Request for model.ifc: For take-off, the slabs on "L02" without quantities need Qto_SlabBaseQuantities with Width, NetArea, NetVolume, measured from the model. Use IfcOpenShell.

First a look at what the model holds.

```python
import ifcopenshell
import ifcopenshell.util.element
import ifcopenshell.util.unit

model = ifcopenshell.open("model.ifc")
print(model.schema)
for unit_type in ("LENGTHUNIT", "AREAUNIT", "VOLUMEUNIT"):
    print(unit_type, ifcopenshell.util.unit.calculate_unit_scale(model, unit_type))
storey = next(s for s in model.by_type("IfcBuildingStorey") if s.Name == "L02")
slabs = [e for e in ifcopenshell.util.element.get_decomposition(storey) if e.is_a("IfcSlab")]
for e in sorted(slabs, key=lambda e: e.id()):
    print(e.id(), e.is_a(), e.Name, list(ifcopenshell.util.element.get_psets(e, qtos_only=True)), sep=" | ")
```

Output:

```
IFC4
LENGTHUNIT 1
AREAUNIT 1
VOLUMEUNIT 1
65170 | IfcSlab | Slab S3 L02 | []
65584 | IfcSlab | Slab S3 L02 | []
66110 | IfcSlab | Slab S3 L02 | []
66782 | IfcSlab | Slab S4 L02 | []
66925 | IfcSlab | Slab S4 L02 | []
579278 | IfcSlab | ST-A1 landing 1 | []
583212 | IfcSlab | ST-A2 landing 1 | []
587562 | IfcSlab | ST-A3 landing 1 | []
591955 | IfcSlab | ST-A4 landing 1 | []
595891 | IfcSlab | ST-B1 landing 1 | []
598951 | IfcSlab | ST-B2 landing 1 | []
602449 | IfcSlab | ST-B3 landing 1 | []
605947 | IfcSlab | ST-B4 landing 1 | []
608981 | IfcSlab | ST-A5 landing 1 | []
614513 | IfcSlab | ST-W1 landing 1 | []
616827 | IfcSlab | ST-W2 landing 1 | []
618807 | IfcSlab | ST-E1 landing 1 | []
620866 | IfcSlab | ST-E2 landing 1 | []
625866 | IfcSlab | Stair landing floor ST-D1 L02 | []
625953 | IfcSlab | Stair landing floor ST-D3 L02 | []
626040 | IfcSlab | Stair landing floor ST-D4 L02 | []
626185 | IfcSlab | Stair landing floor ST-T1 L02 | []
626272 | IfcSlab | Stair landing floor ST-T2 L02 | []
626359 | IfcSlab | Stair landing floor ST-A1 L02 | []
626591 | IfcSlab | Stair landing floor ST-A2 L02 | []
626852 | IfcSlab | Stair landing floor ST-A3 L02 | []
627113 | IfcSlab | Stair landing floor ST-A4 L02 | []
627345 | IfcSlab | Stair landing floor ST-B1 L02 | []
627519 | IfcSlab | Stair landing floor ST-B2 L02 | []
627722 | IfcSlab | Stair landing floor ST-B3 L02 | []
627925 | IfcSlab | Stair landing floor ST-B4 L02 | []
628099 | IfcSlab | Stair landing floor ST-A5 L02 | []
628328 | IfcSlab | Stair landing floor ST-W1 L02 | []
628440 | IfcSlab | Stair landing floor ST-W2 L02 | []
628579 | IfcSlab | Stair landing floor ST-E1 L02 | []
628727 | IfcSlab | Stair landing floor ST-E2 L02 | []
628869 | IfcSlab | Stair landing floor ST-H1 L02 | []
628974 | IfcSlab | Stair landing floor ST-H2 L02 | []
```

```python
import ifcopenshell
import ifcopenshell.api.pset
import ifcopenshell.geom
import ifcopenshell.util.element
import ifcopenshell.util.shape
import ifcopenshell.util.unit

model = ifcopenshell.open("model.ifc")
unit_scale = ifcopenshell.util.unit.calculate_unit_scale(model)
area_scale = ifcopenshell.util.unit.calculate_unit_scale(model, "AREAUNIT")
volume_scale = ifcopenshell.util.unit.calculate_unit_scale(model, "VOLUMEUNIT")
settings = ifcopenshell.geom.settings()

storey = next(s for s in model.by_type("IfcBuildingStorey") if s.Name == "L02")
slabs = [e for e in ifcopenshell.util.element.get_decomposition(storey) if e.is_a("IfcSlab")]

for e in sorted(slabs, key=lambda e: e.id()):
    if ifcopenshell.util.element.get_psets(e, qtos_only=True, should_inherit=False):
        continue
    # Geometry comes back in metres, in the element's own axes.
    shape = ifcopenshell.geom.create_shape(settings, e)
    values = {
        "Width": ifcopenshell.util.shape.get_z(shape.geometry) / unit_scale,
        "NetArea": ifcopenshell.util.shape.get_footprint_area(shape.geometry) / area_scale,
        "NetVolume": ifcopenshell.util.shape.get_volume(shape.geometry) / volume_scale,
    }
    qto = ifcopenshell.api.pset.add_qto(model, product=e, name="Qto_SlabBaseQuantities")
    ifcopenshell.api.pset.edit_qto(model, qto=qto, properties=values)
    print(e.id(), {k: round(v, 3) for k, v in values.items()})

model.write("model_updated.ifc")
```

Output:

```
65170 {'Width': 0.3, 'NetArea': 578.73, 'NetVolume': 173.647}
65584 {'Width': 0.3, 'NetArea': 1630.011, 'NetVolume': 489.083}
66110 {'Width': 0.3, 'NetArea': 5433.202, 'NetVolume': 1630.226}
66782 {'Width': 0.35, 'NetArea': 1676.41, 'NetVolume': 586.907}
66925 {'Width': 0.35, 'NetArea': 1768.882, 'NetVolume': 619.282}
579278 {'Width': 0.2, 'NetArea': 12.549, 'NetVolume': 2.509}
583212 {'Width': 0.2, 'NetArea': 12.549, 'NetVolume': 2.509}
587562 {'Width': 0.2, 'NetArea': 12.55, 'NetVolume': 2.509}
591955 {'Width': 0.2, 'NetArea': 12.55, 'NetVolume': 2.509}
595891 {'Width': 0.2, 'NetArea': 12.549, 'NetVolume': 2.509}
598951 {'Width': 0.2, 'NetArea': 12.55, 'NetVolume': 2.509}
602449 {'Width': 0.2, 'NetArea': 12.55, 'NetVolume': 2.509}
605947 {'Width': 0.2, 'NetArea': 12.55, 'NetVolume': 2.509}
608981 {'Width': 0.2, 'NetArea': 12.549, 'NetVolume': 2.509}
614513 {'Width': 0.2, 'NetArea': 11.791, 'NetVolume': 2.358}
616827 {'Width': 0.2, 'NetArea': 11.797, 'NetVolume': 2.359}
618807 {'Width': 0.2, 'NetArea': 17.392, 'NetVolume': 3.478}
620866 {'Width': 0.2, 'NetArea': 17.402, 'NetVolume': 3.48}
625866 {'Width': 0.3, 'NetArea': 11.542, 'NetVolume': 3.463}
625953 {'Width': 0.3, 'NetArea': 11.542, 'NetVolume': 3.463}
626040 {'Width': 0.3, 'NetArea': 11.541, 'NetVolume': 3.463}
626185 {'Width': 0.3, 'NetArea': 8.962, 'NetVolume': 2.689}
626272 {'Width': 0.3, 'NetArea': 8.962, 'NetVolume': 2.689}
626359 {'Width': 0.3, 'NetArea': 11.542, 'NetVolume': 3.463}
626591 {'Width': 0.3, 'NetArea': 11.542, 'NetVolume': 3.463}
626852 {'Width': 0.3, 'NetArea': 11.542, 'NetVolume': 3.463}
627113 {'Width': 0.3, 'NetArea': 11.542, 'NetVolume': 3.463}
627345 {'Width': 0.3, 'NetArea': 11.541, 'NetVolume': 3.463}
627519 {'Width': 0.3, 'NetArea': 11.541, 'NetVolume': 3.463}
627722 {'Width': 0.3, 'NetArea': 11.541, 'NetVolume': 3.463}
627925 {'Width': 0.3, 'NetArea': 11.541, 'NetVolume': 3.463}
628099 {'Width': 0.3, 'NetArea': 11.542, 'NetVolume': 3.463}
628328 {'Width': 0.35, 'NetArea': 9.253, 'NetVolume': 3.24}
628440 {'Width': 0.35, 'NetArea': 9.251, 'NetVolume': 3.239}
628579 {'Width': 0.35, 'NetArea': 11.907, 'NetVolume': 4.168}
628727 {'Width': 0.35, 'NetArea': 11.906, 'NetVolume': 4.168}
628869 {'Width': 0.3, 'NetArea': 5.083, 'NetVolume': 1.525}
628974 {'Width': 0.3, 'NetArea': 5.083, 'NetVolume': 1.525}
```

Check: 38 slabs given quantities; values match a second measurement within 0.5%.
